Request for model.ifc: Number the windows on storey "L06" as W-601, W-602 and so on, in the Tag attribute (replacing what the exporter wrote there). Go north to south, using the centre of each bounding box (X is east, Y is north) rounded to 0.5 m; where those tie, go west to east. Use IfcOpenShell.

First a look at what the model holds.

```python
import ifcopenshell
import ifcopenshell.util.element
import ifcopenshell.util.placement

model = ifcopenshell.open("model.ifc")
print(model.schema)
storey = next(s for s in model.by_type("IfcBuildingStorey") if s.Name == "L06")
windows = [e for e in ifcopenshell.util.element.get_decomposition(storey) if e.is_a("IfcWindow")]
for e in sorted(windows, key=lambda e: e.id()):
    origin = ifcopenshell.util.placement.get_local_placement(e.ObjectPlacement)[:3, 3]
    print(e.id(), e.Tag, e.Name, origin.round(2) + 0.0, sep=" | ")
```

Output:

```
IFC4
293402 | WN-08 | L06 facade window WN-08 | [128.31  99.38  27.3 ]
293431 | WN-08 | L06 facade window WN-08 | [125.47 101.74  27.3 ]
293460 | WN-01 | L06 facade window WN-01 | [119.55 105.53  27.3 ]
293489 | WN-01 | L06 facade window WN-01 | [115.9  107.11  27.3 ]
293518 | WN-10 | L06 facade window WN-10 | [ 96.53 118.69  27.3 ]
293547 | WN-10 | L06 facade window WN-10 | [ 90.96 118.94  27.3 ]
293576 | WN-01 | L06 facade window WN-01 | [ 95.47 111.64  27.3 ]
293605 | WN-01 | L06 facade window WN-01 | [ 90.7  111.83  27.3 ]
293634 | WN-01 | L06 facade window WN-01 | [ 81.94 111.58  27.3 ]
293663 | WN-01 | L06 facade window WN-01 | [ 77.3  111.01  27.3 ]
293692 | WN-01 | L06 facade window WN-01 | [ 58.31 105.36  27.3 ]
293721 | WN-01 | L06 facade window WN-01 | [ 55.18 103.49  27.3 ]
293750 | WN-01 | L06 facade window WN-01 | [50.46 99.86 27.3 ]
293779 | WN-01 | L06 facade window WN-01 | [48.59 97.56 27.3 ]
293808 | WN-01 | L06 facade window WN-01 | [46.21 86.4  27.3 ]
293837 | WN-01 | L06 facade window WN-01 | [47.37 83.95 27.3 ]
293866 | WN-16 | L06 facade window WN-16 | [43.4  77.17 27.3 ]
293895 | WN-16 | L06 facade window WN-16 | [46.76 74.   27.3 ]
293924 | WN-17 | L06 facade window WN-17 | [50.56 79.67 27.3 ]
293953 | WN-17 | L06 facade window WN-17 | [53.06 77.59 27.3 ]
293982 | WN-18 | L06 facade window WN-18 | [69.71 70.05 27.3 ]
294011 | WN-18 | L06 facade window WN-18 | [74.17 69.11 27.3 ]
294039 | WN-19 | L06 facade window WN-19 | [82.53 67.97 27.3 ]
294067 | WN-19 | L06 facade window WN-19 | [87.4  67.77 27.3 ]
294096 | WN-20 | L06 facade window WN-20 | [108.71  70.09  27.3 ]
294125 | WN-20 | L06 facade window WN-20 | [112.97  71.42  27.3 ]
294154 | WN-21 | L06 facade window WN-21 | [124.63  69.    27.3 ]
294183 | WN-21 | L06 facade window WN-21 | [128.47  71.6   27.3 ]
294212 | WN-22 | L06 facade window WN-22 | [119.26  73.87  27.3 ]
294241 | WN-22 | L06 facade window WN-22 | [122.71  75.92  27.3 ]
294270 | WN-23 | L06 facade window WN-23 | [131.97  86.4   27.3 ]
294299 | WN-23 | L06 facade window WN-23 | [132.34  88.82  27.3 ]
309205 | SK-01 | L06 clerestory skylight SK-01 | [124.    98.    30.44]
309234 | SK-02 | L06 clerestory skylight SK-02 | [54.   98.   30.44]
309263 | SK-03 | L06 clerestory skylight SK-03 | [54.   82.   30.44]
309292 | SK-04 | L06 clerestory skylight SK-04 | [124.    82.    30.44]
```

```python
import ifcopenshell
import ifcopenshell.geom
import ifcopenshell.util.element
import ifcopenshell.util.shape

model = ifcopenshell.open("model.ifc")
settings = ifcopenshell.geom.settings()
settings.set("use-world-coords", True)


def centre(element):
    shape = ifcopenshell.geom.create_shape(settings, element)
    return ifcopenshell.util.shape.get_bbox_centroid(shape.geometry)


storey = next(s for s in model.by_type("IfcBuildingStorey") if s.Name == "L06")
windows = [e for e in ifcopenshell.util.element.get_decomposition(storey) if e.is_a("IfcWindow")]

# Insertion points can sit at a corner or the storey origin, so sort by the geometry (in metres).
centres = {e: centre(e) for e in windows}
windows.sort(key=lambda e: (-round(centres[e][1] / 0.5), centres[e][0]))

for i, e in enumerate(windows, start=1):
    number = f"W-6{i:02d}"
    e.Tag = number
    print(e.id(), number)

model.write("model_updated.ifc")
```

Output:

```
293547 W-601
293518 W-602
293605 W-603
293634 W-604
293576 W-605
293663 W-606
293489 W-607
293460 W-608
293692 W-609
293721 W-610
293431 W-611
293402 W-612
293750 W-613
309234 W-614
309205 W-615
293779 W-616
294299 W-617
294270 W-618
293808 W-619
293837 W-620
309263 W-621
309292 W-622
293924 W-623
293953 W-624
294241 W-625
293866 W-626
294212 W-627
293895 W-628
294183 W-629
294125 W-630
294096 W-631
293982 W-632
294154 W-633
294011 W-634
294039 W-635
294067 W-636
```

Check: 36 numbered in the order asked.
